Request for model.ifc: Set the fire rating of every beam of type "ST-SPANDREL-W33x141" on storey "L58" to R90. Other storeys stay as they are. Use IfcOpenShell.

First a look at what the model holds.

```python
import ifcopenshell
import ifcopenshell.util.element

model = ifcopenshell.open("model.ifc")
print(model.schema)
storey = next(s for s in model.by_type("IfcBuildingStorey") if s.Name == "L58")
beams = [e for e in ifcopenshell.util.element.get_decomposition(storey) if e.is_a("IfcBeam")]
seen = {}
for e in beams:
    element_type = ifcopenshell.util.element.get_type(e)
    key = (element_type.Name if element_type != e and element_type else None, ifcopenshell.util.element.get_pset(e, "Pset_BeamCommon", "FireRating"))
    seen[key] = seen.get(key, 0) + 1
for (name, value), count in sorted(seen.items(), key=str):
    print(count, "x", name, "|", value)
```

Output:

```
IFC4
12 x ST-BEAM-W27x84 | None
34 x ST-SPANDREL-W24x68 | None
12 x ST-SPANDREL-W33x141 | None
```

```python
import ifcopenshell
import ifcopenshell.api.pset
import ifcopenshell.util.element

model = ifcopenshell.open("model.ifc")

storey = next(s for s in model.by_type("IfcBuildingStorey") if s.Name == "L58")
beams = [e for e in ifcopenshell.util.element.get_decomposition(storey) if e.is_a("IfcBeam")]

count = 0
for e in beams:
    element_type = ifcopenshell.util.element.get_type(e)
    if element_type in (None, e) or element_type.Name != "ST-SPANDREL-W33x141":
        continue
    found = ifcopenshell.util.element.get_pset(e, "Pset_BeamCommon", should_inherit=False)
    if found:
        pset = model.by_id(found["id"])
        if len(ifcopenshell.util.element.get_elements_by_pset(pset)) > 1:
            pset = ifcopenshell.api.pset.unshare_pset(model, products=[e], pset=pset)[0]
    else:
        pset = ifcopenshell.api.pset.add_pset(model, product=e, name="Pset_BeamCommon")
    ifcopenshell.api.pset.edit_pset(model, pset=pset, properties={"FireRating": "R90"})
    count += 1

print(count, "beams updated")

model.write("model_updated.ifc")
```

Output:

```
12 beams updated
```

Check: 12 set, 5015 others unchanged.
